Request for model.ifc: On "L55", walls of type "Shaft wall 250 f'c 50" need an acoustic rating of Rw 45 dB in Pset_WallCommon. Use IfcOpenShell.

First a look at what the model holds.

```python
import ifcopenshell
import ifcopenshell.util.element

model = ifcopenshell.open("model.ifc")
print(model.schema)
storey = next(s for s in model.by_type("IfcBuildingStorey") if s.Name == "L55")
walls = [e for e in ifcopenshell.util.element.get_decomposition(storey) if e.is_a("IfcWall")]
seen = {}
for e in walls:
    element_type = ifcopenshell.util.element.get_type(e)
    key = (element_type.Name if element_type != e and element_type else None, ifcopenshell.util.element.get_pset(e, "Pset_WallCommon", "AcousticRating"))
    seen[key] = seen.get(key, 0) + 1
for (name, value), count in sorted(seen.items(), key=str):
    print(count, "x", name, "|", value)
```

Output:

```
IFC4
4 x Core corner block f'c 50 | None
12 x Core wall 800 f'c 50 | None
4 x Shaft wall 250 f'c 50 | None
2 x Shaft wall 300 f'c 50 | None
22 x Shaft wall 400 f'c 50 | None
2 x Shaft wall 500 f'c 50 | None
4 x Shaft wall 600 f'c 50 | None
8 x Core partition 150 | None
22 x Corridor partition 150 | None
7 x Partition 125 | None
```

```python
import ifcopenshell
import ifcopenshell.api.pset
import ifcopenshell.util.element

model = ifcopenshell.open("model.ifc")

storey = next(s for s in model.by_type("IfcBuildingStorey") if s.Name == "L55")
walls = [e for e in ifcopenshell.util.element.get_decomposition(storey) if e.is_a("IfcWall")]

count = 0
for e in walls:
    element_type = ifcopenshell.util.element.get_type(e)
    if element_type in (None, e) or element_type.Name != "Shaft wall 250 f'c 50":
        continue
    # add_pset returns the element's existing set when there is one.
    pset = ifcopenshell.api.pset.add_pset(model, product=e, name="Pset_WallCommon")
    ifcopenshell.api.pset.edit_pset(model, pset=pset, properties={"AcousticRating": "Rw 45 dB"})
    count += 1

print(count, "walls updated")

model.write("model_rev.ifc")
```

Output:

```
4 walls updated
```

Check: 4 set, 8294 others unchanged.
